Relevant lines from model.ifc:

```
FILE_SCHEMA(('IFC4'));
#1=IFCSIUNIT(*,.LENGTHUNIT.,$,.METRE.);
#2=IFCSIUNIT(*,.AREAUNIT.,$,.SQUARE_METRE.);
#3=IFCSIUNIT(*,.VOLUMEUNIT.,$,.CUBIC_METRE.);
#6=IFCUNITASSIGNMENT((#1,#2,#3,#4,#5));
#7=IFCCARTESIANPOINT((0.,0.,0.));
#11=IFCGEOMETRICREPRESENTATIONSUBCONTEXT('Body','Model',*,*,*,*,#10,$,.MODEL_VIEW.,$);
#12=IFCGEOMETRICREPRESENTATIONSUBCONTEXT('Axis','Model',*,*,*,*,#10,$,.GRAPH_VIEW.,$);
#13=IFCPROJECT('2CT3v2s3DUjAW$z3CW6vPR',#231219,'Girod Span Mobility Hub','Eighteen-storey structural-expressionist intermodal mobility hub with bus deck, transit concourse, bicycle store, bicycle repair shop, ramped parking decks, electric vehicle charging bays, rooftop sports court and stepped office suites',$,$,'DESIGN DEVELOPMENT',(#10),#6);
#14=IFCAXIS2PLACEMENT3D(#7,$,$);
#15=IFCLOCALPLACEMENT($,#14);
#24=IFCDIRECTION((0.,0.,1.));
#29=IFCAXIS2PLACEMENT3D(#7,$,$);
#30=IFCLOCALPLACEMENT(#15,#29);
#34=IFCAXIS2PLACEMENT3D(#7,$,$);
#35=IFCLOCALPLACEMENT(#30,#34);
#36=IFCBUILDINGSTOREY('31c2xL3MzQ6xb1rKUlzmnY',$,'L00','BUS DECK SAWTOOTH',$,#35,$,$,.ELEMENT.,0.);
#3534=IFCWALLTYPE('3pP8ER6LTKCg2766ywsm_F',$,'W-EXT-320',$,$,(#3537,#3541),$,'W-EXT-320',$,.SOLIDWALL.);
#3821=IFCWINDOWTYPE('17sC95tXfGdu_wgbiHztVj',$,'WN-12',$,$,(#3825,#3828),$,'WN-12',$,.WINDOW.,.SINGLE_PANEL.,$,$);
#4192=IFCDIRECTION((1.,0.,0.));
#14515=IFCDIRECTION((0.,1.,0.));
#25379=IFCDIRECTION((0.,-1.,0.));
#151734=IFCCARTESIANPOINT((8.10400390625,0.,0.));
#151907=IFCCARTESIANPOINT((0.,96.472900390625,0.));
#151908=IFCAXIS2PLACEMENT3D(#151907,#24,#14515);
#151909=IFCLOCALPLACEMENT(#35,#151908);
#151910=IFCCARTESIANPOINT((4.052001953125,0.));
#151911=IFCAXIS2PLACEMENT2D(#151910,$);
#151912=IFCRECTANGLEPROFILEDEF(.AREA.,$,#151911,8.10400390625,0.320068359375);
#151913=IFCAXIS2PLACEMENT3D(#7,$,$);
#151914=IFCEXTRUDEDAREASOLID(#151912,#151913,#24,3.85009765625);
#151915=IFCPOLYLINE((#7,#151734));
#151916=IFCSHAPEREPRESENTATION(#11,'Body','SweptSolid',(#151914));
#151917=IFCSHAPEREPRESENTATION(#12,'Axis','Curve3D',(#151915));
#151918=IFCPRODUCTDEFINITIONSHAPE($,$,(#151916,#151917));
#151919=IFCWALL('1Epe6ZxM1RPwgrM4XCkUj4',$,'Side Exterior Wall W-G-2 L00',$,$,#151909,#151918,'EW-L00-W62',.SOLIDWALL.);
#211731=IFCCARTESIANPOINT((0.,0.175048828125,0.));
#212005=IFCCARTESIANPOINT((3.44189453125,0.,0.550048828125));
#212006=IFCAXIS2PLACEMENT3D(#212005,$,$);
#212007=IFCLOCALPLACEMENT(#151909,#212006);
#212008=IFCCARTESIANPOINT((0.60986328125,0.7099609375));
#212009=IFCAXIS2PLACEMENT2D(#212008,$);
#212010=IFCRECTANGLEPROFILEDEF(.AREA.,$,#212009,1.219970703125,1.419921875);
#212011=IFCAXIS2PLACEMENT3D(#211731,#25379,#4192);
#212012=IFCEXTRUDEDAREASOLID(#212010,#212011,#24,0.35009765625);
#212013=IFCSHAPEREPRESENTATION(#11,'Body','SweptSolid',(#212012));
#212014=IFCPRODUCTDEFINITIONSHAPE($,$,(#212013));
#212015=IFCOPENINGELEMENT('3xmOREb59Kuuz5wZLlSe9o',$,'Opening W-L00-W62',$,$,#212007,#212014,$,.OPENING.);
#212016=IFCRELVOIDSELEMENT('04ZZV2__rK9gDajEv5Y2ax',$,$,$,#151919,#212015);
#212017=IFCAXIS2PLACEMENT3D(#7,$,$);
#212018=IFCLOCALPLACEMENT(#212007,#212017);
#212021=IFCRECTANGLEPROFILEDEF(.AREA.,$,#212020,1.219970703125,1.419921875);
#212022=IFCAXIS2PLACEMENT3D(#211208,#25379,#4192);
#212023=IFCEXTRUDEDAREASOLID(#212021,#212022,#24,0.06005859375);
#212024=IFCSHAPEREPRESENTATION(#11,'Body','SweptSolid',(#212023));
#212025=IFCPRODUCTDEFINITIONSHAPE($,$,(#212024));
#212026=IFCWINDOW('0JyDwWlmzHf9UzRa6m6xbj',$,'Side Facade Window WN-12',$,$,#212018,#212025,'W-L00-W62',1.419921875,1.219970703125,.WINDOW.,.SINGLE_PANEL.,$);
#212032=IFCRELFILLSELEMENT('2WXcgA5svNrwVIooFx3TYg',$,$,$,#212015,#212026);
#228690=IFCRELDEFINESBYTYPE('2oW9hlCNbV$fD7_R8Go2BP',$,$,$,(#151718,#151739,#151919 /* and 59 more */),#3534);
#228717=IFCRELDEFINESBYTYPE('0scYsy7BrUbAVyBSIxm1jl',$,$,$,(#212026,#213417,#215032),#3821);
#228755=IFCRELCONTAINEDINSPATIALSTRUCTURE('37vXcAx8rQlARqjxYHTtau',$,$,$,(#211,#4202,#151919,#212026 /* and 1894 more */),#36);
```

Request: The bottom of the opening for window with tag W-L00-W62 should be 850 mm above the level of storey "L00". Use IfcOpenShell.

```python
import numpy as np
import ifcopenshell
import ifcopenshell.api.geometry
import ifcopenshell.geom
import ifcopenshell.util.element
import ifcopenshell.util.placement
import ifcopenshell.util.shape
import ifcopenshell.util.unit

model = ifcopenshell.open("model.ifc")
unit_scale = ifcopenshell.util.unit.calculate_unit_scale(model)

window = model.by_guid("0JyDwWlmzHf9UzRa6m6xbj")
opening = window.FillsVoids[0].RelatingOpeningElement
storey = ifcopenshell.util.element.get_container(window, ifc_class="IfcBuildingStorey")
level = ifcopenshell.util.placement.get_local_placement(storey.ObjectPlacement)[2, 3]

# The opening's origin need not be at the sill, so measure its lowest point.
shape = ifcopenshell.geom.create_shape(ifcopenshell.geom.settings(), opening)
bottom = ifcopenshell.util.shape.get_shape_bottom_elevation(shape, shape.geometry) / unit_scale
dz = level + 0.85 / unit_scale - bottom

shift = np.array([0.0, 0.0, dz])
# The window is placed relative to its opening, so it follows when the opening moves.
matrix = ifcopenshell.util.placement.get_local_placement(opening.ObjectPlacement)
matrix[:3, 3] += shift
ifcopenshell.api.geometry.edit_object_placement(
    model, product=opening, matrix=matrix, is_si=False, should_transform_children=True
)

print(f"moved by {dz * unit_scale:+.3f} m")

model.write("model_updated.ifc")
```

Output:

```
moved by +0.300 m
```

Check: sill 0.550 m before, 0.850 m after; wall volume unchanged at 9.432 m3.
